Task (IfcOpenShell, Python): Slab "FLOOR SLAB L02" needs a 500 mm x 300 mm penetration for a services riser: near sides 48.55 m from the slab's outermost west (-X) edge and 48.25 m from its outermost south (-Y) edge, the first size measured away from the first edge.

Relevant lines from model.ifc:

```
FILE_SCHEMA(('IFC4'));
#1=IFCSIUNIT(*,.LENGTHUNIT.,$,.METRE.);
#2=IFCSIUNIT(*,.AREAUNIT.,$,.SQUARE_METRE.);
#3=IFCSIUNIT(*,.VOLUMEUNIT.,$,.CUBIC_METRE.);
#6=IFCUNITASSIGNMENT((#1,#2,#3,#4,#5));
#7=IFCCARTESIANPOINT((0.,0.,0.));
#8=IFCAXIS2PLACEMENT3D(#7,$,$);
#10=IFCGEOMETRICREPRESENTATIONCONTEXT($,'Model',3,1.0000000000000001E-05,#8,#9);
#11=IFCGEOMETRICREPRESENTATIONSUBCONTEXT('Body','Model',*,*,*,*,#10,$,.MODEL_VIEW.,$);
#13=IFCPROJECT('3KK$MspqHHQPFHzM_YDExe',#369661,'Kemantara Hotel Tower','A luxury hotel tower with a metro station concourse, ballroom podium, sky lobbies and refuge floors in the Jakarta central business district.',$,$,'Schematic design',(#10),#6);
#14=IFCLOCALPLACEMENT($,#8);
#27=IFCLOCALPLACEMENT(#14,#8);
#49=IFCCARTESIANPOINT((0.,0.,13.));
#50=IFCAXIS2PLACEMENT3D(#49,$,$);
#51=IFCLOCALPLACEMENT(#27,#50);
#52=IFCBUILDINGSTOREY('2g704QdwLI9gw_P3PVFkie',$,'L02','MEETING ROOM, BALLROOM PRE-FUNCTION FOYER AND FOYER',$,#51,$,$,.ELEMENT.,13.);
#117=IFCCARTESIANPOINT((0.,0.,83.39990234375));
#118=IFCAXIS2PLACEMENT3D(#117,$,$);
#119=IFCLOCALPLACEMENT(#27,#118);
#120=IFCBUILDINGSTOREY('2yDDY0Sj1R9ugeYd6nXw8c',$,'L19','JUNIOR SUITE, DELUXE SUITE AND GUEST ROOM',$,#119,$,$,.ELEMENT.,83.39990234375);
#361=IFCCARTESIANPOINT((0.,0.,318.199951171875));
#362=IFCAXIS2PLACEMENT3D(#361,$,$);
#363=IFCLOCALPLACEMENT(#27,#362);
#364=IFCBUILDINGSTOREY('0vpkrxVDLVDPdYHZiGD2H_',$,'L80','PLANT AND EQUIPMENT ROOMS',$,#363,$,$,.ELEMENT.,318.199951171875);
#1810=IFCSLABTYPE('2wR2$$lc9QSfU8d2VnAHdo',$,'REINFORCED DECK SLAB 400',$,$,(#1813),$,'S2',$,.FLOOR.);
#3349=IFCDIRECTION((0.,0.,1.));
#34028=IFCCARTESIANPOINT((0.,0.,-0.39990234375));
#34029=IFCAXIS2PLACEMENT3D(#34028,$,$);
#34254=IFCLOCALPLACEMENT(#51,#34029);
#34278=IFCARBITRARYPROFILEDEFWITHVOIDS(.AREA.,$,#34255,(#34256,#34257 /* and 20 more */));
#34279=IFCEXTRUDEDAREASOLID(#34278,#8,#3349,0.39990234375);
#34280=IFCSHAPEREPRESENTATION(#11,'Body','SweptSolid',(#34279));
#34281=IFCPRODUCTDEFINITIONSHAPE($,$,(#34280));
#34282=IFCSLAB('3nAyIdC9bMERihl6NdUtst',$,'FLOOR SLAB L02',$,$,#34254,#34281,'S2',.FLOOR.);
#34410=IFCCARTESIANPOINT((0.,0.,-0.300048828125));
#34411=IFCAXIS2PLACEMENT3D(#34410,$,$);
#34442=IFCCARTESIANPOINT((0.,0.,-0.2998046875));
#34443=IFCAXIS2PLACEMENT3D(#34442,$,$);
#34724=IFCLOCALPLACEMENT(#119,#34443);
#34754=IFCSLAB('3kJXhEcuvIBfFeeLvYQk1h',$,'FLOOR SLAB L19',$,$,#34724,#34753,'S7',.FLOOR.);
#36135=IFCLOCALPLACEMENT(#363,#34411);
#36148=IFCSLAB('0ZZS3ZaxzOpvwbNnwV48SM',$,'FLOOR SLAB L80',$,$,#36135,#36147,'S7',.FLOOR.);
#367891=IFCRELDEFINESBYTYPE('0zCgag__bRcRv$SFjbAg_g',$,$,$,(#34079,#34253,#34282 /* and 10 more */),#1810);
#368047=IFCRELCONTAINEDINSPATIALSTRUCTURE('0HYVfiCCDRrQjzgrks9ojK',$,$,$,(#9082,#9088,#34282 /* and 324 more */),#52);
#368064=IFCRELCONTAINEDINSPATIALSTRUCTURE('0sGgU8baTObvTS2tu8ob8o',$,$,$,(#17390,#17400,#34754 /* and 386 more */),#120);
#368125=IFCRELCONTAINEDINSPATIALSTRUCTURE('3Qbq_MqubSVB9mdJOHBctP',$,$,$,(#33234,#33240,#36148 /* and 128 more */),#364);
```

```python
import numpy as np
import ifcopenshell
import ifcopenshell.api.feature
import ifcopenshell.api.geometry
import ifcopenshell.api.root
import ifcopenshell.geom
import ifcopenshell.util.placement
import ifcopenshell.util.representation
import ifcopenshell.util.shape
import ifcopenshell.util.unit

model = ifcopenshell.open("model.ifc")
unit_scale = ifcopenshell.util.unit.calculate_unit_scale(model)
settings = ifcopenshell.geom.settings()


def volume(element):
    """Net volume in cubic metres, openings subtracted."""
    shape = ifcopenshell.geom.create_shape(settings, element)
    return ifcopenshell.util.shape.get_volume(shape.geometry)


slab = model.by_guid("3nAyIdC9bMERihl6NdUtst")
before = volume(slab)

# Extent in the slab's own axes, in metres. The edges named are its -X and -Y sides.
slab_shape = ifcopenshell.geom.create_shape(settings, slab)
vertices = ifcopenshell.util.shape.get_vertices(slab_shape.geometry)
x_min, y_min, bottom = vertices.min(axis=0)
top = vertices[:, 2].max()

opening = ifcopenshell.api.root.create_entity(model, ifc_class="IfcOpeningElement", name="Services riser opening", predefined_type="OPENING")
context = ifcopenshell.util.representation.get_context(model, "Model", "Body", "MODEL_VIEW")
width, depth = 0.5, 0.3
outline = [(0.0, 0.0), (width, 0.0), (width, depth), (0.0, depth), (0.0, 0.0)]
# Overshoot both faces by 50 mm so the cut is clean.
shape = ifcopenshell.api.geometry.add_slab_representation(
    model, context=context, depth=top - bottom + 0.1, polyline=outline
)
ifcopenshell.api.geometry.assign_representation(model, product=opening, representation=shape)

matrix = ifcopenshell.util.placement.get_local_placement(slab.ObjectPlacement)
matrix[:, 3] = matrix @ np.append(np.array([x_min + 48.55, y_min + 48.25, bottom - 0.05]) / unit_scale, 1.0)
ifcopenshell.api.geometry.edit_object_placement(model, product=opening, matrix=matrix, is_si=False)
ifcopenshell.api.feature.add_feature(model, feature=opening, element=slab)

after = volume(slab)

print(f"slab volume {before:.3f} -> {after:.3f} m3")

model.write("model_rev.ifc")
```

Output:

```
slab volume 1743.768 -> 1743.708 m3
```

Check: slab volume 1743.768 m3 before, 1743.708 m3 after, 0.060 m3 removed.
